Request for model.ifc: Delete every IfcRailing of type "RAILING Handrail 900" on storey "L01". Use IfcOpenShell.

First a look at what the model holds.

```python
import ifcopenshell
import ifcopenshell.util.element

model = ifcopenshell.open("model.ifc")
print(model.schema)
storey = next(s for s in model.by_type("IfcBuildingStorey") if s.Name == "L01")
railings = [e for e in ifcopenshell.util.element.get_decomposition(storey) if e.is_a("IfcRailing")]
seen = {}
for e in railings:
    element_type = ifcopenshell.util.element.get_type(e)
    name = element_type.Name if element_type not in (None, e) else None
    seen[name] = seen.get(name, 0) + 1
for name, count in sorted(seen.items(), key=str):
    print(count, "x", name)
```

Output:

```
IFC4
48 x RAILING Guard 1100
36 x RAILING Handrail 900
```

```python
import ifcopenshell
import ifcopenshell.api.root
import ifcopenshell.util.element

model = ifcopenshell.open("model.ifc")

storey = next(s for s in model.by_type("IfcBuildingStorey") if s.Name == "L01")
railings = [e for e in ifcopenshell.util.element.get_decomposition(storey) if e.is_a("IfcRailing")]
targets = [e for e in railings if (t := ifcopenshell.util.element.get_type(e)) not in (None, e) and t.Name == "RAILING Handrail 900"]

for e in targets:
    ifcopenshell.api.root.remove_product(model, product=e)
print(len(targets), "removed")

model.write("model_updated.ifc")
```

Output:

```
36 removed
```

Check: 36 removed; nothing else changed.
